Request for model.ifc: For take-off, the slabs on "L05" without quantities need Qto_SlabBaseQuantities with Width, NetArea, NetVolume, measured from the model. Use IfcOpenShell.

First a look at what the model holds.

```python
import ifcopenshell
import ifcopenshell.util.element
import ifcopenshell.util.unit

model = ifcopenshell.open("model.ifc")
print(model.schema)
for unit_type in ("LENGTHUNIT", "AREAUNIT", "VOLUMEUNIT"):
    print(unit_type, ifcopenshell.util.unit.calculate_unit_scale(model, unit_type))
storey = next(s for s in model.by_type("IfcBuildingStorey") if s.Name == "L05")
slabs = [e for e in ifcopenshell.util.element.get_decomposition(storey) if e.is_a("IfcSlab")]
for e in sorted(slabs, key=lambda e: e.id()):
    print(e.id(), e.is_a(), e.Name, list(ifcopenshell.util.element.get_psets(e, qtos_only=True)), sep=" | ")
```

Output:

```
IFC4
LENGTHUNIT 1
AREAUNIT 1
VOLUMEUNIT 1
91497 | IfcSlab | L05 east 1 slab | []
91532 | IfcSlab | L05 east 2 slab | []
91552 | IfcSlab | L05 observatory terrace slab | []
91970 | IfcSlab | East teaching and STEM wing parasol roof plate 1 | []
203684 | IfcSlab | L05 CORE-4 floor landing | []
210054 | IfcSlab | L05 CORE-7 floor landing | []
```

```python
import ifcopenshell
import ifcopenshell.api.pset
import ifcopenshell.geom
import ifcopenshell.util.element
import ifcopenshell.util.shape
import ifcopenshell.util.unit

model = ifcopenshell.open("model.ifc")
unit_scale = ifcopenshell.util.unit.calculate_unit_scale(model)
area_scale = ifcopenshell.util.unit.calculate_unit_scale(model, "AREAUNIT")
volume_scale = ifcopenshell.util.unit.calculate_unit_scale(model, "VOLUMEUNIT")
settings = ifcopenshell.geom.settings()

storey = next(s for s in model.by_type("IfcBuildingStorey") if s.Name == "L05")
slabs = [e for e in ifcopenshell.util.element.get_decomposition(storey) if e.is_a("IfcSlab")]

for e in sorted(slabs, key=lambda e: e.id()):
    if ifcopenshell.util.element.get_psets(e, qtos_only=True, should_inherit=False):
        continue
    # Geometry comes back in metres, in the element's own axes.
    shape = ifcopenshell.geom.create_shape(settings, e)
    values = {
        "Width": ifcopenshell.util.shape.get_z(shape.geometry) / unit_scale,
        "NetArea": ifcopenshell.util.shape.get_footprint_area(shape.geometry) / area_scale,
        "NetVolume": ifcopenshell.util.shape.get_volume(shape.geometry) / volume_scale,
    }
    qto = ifcopenshell.api.pset.add_qto(model, product=e, name="Qto_SlabBaseQuantities")
    ifcopenshell.api.pset.edit_qto(model, qto=qto, properties=values)
    print(e.id(), {k: round(v, 3) for k, v in values.items()})

model.write("model-out.ifc")
```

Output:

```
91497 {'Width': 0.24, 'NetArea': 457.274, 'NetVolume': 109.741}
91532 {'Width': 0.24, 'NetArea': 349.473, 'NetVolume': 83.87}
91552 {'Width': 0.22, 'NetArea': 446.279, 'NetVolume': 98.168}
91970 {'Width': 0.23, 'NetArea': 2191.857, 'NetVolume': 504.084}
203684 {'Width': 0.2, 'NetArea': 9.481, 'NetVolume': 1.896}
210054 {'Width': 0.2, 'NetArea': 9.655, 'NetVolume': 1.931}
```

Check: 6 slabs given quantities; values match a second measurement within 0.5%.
